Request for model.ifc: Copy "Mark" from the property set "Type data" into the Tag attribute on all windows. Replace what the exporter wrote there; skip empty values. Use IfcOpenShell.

First a look at what the model holds.

```python
import ifcopenshell
import ifcopenshell.util.element

model = ifcopenshell.open("model.ifc")
print(model.schema)
windows = model.by_type("IfcWindow")
print(len(windows), "windows")
for e in windows[:8]:
    source = ifcopenshell.util.element.get_pset(e, "Type data", "Mark")
    target = e.Tag
    print(e.id(), repr(source), repr(target), sep=" | ")
```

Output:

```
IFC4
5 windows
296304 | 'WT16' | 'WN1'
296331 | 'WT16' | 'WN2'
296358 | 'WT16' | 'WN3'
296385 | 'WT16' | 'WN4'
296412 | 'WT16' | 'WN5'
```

```python
import ifcopenshell
import ifcopenshell.util.element

model = ifcopenshell.open("model.ifc")

count = 0
for e in model.by_type("IfcWindow"):
    value = ifcopenshell.util.element.get_pset(e, "Type data", "Mark")
    current = e.Tag
    if not value or not value.strip() or current == value:
        continue
    e.Tag = value
    count += 1

print(count, "windows updated")

model.write("model_updated.ifc")
```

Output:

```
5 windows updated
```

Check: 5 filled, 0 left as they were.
